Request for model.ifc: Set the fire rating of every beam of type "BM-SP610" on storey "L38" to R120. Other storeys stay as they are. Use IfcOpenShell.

First a look at what the model holds.

```python
import ifcopenshell
import ifcopenshell.util.element

model = ifcopenshell.open("model.ifc")
print(model.schema)
storey = next(s for s in model.by_type("IfcBuildingStorey") if s.Name == "L38")
beams = [e for e in ifcopenshell.util.element.get_decomposition(storey) if e.is_a("IfcBeam")]
seen = {}
for e in beams:
    element_type = ifcopenshell.util.element.get_type(e)
    key = (element_type.Name if element_type != e and element_type else None, ifcopenshell.util.element.get_pset(e, "Pset_BeamCommon", "FireRating"))
    seen[key] = seen.get(key, 0) + 1
for (name, value), count in sorted(seen.items(), key=str):
    print(count, "x", name, "|", value)
```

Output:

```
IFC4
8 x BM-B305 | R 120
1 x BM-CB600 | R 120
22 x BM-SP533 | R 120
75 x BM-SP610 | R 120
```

```python
import ifcopenshell
import ifcopenshell.api.pset
import ifcopenshell.util.element

model = ifcopenshell.open("model.ifc")

storey = next(s for s in model.by_type("IfcBuildingStorey") if s.Name == "L38")
beams = [e for e in ifcopenshell.util.element.get_decomposition(storey) if e.is_a("IfcBeam")]

count = 0
for e in beams:
    element_type = ifcopenshell.util.element.get_type(e)
    if element_type in (None, e) or element_type.Name != "BM-SP610":
        continue
    found = ifcopenshell.util.element.get_pset(e, "Pset_BeamCommon", should_inherit=False)
    if found:
        pset = model.by_id(found["id"])
        if len(ifcopenshell.util.element.get_elements_by_pset(pset)) > 1:
            pset = ifcopenshell.api.pset.unshare_pset(model, products=[e], pset=pset)[0]
    else:
        pset = ifcopenshell.api.pset.add_pset(model, product=e, name="Pset_BeamCommon")
    ifcopenshell.api.pset.edit_pset(model, pset=pset, properties={"FireRating": "R120"})
    count += 1

print(count, "beams updated")

model.write("model_edited.ifc")
```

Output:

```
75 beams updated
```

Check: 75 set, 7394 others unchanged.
